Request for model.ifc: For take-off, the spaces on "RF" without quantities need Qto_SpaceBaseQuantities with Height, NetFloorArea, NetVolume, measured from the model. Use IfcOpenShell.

First a look at what the model holds.

```python
import ifcopenshell
import ifcopenshell.util.element
import ifcopenshell.util.unit

model = ifcopenshell.open("model.ifc")
print(model.schema)
for unit_type in ("LENGTHUNIT", "AREAUNIT", "VOLUMEUNIT"):
    print(unit_type, ifcopenshell.util.unit.calculate_unit_scale(model, unit_type))
storey = next(s for s in model.by_type("IfcBuildingStorey") if s.Name == "RF")
spaces = [e for e in ifcopenshell.util.element.get_decomposition(storey) if e.is_a("IfcSpace")]
for e in sorted(spaces, key=lambda e: e.id()):
    print(e.id(), e.is_a(), e.Name, list(ifcopenshell.util.element.get_psets(e, qtos_only=True)), sep=" | ")
```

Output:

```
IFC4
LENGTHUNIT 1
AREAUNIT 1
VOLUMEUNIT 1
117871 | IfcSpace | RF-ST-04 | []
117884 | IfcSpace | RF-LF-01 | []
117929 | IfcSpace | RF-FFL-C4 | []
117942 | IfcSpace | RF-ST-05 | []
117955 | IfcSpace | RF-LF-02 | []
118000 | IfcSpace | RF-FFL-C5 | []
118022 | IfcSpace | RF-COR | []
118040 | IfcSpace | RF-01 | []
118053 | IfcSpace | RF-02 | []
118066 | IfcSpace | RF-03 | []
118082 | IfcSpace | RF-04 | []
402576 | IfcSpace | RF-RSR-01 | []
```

```python
import ifcopenshell
import ifcopenshell.api.pset
import ifcopenshell.geom
import ifcopenshell.util.element
import ifcopenshell.util.shape
import ifcopenshell.util.unit

model = ifcopenshell.open("model.ifc")
unit_scale = ifcopenshell.util.unit.calculate_unit_scale(model)
area_scale = ifcopenshell.util.unit.calculate_unit_scale(model, "AREAUNIT")
volume_scale = ifcopenshell.util.unit.calculate_unit_scale(model, "VOLUMEUNIT")
settings = ifcopenshell.geom.settings()

storey = next(s for s in model.by_type("IfcBuildingStorey") if s.Name == "RF")
spaces = [e for e in ifcopenshell.util.element.get_decomposition(storey) if e.is_a("IfcSpace")]

for e in sorted(spaces, key=lambda e: e.id()):
    if ifcopenshell.util.element.get_psets(e, qtos_only=True, should_inherit=False):
        continue
    # Geometry comes back in metres, in the element's own axes.
    shape = ifcopenshell.geom.create_shape(settings, e)
    values = {
        "Height": ifcopenshell.util.shape.get_z(shape.geometry) / unit_scale,
        "NetFloorArea": ifcopenshell.util.shape.get_footprint_area(shape.geometry) / area_scale,
        "NetVolume": ifcopenshell.util.shape.get_volume(shape.geometry) / volume_scale,
    }
    qto = ifcopenshell.api.pset.add_qto(model, product=e, name="Qto_SpaceBaseQuantities")
    ifcopenshell.api.pset.edit_qto(model, qto=qto, properties=values)
    print(e.id(), {k: round(v, 3) for k, v in values.items()})

model.write("model_updated.ifc")
```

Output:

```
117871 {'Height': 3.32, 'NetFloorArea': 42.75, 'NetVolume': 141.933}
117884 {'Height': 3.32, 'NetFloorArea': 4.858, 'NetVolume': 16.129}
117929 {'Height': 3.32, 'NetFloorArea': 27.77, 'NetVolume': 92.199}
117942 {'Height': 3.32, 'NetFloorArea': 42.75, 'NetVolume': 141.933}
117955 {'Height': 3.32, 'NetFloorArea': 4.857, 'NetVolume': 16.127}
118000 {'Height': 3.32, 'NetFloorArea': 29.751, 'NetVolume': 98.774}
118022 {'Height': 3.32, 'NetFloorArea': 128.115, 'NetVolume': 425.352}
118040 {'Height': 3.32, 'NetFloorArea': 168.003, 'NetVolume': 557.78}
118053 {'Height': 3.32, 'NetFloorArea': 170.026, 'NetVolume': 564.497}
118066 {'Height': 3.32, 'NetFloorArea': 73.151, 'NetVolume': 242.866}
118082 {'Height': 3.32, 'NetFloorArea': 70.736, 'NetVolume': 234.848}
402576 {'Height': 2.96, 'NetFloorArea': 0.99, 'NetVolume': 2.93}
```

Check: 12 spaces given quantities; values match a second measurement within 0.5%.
